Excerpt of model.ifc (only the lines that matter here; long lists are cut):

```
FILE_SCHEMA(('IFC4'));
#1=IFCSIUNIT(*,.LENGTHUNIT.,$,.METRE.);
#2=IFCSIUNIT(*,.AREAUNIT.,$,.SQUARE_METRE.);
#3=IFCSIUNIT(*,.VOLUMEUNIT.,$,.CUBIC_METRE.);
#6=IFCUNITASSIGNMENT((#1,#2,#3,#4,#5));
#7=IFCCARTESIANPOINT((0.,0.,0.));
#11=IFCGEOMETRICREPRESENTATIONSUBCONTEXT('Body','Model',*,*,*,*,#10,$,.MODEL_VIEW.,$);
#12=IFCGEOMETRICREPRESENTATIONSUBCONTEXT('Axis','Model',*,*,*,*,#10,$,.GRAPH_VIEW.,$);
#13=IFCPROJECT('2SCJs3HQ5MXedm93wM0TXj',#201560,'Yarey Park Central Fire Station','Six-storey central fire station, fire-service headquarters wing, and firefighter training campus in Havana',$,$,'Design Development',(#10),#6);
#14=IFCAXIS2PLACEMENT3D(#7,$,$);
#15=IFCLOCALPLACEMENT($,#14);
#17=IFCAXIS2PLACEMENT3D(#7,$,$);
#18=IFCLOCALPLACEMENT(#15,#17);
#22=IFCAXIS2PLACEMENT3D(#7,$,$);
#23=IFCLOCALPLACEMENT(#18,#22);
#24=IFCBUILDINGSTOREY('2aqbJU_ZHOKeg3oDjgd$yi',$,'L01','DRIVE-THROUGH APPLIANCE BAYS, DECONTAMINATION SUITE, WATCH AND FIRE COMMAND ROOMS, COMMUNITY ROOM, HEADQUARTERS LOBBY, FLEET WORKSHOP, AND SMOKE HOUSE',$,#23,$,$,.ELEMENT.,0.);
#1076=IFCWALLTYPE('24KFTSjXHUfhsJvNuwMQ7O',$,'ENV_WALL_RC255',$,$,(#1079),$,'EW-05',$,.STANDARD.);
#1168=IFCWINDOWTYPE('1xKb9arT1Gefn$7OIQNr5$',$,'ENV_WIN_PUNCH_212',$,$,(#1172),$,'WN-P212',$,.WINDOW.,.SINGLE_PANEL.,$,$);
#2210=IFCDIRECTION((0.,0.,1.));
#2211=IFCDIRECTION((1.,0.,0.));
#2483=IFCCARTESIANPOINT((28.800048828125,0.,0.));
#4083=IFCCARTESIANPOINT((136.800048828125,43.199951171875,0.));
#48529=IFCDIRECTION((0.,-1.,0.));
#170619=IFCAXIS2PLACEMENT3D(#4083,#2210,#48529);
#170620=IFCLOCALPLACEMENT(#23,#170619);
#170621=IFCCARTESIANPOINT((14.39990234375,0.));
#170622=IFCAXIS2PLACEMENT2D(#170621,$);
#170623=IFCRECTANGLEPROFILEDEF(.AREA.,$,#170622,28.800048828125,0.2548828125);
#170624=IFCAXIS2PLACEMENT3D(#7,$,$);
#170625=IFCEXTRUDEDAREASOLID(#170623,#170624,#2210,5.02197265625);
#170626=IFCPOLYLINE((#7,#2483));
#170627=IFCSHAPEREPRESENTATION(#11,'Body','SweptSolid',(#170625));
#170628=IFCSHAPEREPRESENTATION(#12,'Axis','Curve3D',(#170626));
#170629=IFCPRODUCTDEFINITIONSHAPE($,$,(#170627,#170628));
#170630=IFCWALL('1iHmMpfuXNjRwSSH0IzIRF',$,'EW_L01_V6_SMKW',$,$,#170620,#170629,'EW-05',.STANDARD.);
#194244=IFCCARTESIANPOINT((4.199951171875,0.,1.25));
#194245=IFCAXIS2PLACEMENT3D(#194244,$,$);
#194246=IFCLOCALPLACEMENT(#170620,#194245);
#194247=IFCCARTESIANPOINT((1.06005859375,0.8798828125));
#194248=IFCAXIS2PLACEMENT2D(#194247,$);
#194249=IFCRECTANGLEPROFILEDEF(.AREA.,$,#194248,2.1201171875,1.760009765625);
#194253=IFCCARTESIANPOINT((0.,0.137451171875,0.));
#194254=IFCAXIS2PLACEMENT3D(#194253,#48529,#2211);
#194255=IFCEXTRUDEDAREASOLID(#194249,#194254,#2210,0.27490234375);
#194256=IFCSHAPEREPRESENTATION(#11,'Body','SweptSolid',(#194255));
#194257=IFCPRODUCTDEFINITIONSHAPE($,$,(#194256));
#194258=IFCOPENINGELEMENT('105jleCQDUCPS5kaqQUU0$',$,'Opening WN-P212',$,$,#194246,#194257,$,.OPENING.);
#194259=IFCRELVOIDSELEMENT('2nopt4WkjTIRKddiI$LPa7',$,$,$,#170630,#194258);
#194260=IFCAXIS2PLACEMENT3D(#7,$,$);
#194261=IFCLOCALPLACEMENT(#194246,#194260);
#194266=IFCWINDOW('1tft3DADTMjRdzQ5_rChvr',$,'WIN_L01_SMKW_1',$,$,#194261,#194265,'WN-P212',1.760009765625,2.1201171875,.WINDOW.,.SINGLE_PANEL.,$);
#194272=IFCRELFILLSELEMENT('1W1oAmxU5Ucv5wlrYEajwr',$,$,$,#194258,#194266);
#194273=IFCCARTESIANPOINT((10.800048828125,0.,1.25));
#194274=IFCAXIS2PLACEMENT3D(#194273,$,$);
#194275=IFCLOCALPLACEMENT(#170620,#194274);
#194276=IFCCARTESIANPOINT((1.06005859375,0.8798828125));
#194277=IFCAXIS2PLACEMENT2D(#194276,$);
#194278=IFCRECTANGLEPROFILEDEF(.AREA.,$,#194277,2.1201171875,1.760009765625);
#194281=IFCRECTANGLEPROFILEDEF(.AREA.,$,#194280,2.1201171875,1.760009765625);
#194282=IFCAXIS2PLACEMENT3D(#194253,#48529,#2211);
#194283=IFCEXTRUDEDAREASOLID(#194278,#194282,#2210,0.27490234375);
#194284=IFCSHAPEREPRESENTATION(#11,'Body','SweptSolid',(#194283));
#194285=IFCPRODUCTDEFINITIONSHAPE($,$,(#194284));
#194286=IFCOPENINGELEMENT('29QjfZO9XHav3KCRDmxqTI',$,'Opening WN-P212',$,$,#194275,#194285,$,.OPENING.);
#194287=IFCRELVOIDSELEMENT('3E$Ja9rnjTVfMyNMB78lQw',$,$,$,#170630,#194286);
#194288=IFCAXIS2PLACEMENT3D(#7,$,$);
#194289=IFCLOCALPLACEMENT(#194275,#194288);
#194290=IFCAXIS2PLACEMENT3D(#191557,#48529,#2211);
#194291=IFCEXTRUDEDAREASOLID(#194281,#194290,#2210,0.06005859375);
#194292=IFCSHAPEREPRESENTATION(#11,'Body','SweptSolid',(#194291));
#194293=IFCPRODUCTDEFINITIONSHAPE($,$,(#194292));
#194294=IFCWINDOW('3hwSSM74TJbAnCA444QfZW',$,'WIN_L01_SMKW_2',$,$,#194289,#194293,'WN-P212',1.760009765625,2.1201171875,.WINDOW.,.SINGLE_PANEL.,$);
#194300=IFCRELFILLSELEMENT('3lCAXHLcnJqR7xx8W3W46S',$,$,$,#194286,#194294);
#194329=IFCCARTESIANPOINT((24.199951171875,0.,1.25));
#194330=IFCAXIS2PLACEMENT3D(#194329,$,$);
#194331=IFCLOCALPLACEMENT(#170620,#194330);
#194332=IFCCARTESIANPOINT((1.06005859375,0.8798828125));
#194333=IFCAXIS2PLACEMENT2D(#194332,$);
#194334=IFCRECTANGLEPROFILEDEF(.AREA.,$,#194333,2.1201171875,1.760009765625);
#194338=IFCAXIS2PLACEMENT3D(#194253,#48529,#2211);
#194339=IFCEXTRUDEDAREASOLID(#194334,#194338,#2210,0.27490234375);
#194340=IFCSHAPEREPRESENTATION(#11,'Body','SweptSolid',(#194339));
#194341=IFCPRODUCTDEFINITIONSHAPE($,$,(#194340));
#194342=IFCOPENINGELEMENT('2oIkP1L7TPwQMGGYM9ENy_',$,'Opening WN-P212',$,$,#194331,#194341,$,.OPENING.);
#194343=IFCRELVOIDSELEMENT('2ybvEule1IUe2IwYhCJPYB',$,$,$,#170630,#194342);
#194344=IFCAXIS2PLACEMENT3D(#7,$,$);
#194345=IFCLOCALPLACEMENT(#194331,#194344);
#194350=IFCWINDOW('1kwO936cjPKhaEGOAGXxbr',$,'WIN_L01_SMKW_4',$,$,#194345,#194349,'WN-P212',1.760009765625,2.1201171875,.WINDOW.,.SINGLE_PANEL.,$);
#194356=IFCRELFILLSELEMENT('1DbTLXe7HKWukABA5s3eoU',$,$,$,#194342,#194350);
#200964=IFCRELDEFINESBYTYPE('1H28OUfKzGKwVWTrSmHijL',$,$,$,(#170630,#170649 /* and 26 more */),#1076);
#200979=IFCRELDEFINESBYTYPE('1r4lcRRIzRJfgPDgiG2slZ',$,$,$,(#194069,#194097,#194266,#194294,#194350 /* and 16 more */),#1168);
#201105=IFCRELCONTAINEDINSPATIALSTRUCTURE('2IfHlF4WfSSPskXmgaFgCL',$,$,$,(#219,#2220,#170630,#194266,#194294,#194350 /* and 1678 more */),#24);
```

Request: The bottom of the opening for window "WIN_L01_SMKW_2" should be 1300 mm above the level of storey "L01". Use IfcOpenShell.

```python
import numpy as np
import ifcopenshell
import ifcopenshell.api.geometry
import ifcopenshell.geom
import ifcopenshell.util.element
import ifcopenshell.util.placement
import ifcopenshell.util.shape
import ifcopenshell.util.unit

model = ifcopenshell.open("model.ifc")
unit_scale = ifcopenshell.util.unit.calculate_unit_scale(model)

window = model.by_guid("3hwSSM74TJbAnCA444QfZW")
opening = window.FillsVoids[0].RelatingOpeningElement
storey = ifcopenshell.util.element.get_container(window, ifc_class="IfcBuildingStorey")
level = ifcopenshell.util.placement.get_local_placement(storey.ObjectPlacement)[2, 3]

# The opening's origin need not be at the sill, so measure its lowest point.
shape = ifcopenshell.geom.create_shape(ifcopenshell.geom.settings(), opening)
bottom = ifcopenshell.util.shape.get_shape_bottom_elevation(shape, shape.geometry) / unit_scale
dz = level + 1.3 - bottom

shift = np.array([0.0, 0.0, dz])
# The window is placed relative to its opening, so it follows when the opening moves.
matrix = ifcopenshell.util.placement.get_local_placement(opening.ObjectPlacement)
matrix[:3, 3] += shift
ifcopenshell.api.geometry.edit_object_placement(
    model, product=opening, matrix=matrix, is_si=False, should_transform_children=True
)

print(f"moved by {dz * unit_scale:+.3f} m")

model.write("model_v2.ifc")
```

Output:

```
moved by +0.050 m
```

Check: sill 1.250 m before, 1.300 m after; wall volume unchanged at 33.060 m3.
